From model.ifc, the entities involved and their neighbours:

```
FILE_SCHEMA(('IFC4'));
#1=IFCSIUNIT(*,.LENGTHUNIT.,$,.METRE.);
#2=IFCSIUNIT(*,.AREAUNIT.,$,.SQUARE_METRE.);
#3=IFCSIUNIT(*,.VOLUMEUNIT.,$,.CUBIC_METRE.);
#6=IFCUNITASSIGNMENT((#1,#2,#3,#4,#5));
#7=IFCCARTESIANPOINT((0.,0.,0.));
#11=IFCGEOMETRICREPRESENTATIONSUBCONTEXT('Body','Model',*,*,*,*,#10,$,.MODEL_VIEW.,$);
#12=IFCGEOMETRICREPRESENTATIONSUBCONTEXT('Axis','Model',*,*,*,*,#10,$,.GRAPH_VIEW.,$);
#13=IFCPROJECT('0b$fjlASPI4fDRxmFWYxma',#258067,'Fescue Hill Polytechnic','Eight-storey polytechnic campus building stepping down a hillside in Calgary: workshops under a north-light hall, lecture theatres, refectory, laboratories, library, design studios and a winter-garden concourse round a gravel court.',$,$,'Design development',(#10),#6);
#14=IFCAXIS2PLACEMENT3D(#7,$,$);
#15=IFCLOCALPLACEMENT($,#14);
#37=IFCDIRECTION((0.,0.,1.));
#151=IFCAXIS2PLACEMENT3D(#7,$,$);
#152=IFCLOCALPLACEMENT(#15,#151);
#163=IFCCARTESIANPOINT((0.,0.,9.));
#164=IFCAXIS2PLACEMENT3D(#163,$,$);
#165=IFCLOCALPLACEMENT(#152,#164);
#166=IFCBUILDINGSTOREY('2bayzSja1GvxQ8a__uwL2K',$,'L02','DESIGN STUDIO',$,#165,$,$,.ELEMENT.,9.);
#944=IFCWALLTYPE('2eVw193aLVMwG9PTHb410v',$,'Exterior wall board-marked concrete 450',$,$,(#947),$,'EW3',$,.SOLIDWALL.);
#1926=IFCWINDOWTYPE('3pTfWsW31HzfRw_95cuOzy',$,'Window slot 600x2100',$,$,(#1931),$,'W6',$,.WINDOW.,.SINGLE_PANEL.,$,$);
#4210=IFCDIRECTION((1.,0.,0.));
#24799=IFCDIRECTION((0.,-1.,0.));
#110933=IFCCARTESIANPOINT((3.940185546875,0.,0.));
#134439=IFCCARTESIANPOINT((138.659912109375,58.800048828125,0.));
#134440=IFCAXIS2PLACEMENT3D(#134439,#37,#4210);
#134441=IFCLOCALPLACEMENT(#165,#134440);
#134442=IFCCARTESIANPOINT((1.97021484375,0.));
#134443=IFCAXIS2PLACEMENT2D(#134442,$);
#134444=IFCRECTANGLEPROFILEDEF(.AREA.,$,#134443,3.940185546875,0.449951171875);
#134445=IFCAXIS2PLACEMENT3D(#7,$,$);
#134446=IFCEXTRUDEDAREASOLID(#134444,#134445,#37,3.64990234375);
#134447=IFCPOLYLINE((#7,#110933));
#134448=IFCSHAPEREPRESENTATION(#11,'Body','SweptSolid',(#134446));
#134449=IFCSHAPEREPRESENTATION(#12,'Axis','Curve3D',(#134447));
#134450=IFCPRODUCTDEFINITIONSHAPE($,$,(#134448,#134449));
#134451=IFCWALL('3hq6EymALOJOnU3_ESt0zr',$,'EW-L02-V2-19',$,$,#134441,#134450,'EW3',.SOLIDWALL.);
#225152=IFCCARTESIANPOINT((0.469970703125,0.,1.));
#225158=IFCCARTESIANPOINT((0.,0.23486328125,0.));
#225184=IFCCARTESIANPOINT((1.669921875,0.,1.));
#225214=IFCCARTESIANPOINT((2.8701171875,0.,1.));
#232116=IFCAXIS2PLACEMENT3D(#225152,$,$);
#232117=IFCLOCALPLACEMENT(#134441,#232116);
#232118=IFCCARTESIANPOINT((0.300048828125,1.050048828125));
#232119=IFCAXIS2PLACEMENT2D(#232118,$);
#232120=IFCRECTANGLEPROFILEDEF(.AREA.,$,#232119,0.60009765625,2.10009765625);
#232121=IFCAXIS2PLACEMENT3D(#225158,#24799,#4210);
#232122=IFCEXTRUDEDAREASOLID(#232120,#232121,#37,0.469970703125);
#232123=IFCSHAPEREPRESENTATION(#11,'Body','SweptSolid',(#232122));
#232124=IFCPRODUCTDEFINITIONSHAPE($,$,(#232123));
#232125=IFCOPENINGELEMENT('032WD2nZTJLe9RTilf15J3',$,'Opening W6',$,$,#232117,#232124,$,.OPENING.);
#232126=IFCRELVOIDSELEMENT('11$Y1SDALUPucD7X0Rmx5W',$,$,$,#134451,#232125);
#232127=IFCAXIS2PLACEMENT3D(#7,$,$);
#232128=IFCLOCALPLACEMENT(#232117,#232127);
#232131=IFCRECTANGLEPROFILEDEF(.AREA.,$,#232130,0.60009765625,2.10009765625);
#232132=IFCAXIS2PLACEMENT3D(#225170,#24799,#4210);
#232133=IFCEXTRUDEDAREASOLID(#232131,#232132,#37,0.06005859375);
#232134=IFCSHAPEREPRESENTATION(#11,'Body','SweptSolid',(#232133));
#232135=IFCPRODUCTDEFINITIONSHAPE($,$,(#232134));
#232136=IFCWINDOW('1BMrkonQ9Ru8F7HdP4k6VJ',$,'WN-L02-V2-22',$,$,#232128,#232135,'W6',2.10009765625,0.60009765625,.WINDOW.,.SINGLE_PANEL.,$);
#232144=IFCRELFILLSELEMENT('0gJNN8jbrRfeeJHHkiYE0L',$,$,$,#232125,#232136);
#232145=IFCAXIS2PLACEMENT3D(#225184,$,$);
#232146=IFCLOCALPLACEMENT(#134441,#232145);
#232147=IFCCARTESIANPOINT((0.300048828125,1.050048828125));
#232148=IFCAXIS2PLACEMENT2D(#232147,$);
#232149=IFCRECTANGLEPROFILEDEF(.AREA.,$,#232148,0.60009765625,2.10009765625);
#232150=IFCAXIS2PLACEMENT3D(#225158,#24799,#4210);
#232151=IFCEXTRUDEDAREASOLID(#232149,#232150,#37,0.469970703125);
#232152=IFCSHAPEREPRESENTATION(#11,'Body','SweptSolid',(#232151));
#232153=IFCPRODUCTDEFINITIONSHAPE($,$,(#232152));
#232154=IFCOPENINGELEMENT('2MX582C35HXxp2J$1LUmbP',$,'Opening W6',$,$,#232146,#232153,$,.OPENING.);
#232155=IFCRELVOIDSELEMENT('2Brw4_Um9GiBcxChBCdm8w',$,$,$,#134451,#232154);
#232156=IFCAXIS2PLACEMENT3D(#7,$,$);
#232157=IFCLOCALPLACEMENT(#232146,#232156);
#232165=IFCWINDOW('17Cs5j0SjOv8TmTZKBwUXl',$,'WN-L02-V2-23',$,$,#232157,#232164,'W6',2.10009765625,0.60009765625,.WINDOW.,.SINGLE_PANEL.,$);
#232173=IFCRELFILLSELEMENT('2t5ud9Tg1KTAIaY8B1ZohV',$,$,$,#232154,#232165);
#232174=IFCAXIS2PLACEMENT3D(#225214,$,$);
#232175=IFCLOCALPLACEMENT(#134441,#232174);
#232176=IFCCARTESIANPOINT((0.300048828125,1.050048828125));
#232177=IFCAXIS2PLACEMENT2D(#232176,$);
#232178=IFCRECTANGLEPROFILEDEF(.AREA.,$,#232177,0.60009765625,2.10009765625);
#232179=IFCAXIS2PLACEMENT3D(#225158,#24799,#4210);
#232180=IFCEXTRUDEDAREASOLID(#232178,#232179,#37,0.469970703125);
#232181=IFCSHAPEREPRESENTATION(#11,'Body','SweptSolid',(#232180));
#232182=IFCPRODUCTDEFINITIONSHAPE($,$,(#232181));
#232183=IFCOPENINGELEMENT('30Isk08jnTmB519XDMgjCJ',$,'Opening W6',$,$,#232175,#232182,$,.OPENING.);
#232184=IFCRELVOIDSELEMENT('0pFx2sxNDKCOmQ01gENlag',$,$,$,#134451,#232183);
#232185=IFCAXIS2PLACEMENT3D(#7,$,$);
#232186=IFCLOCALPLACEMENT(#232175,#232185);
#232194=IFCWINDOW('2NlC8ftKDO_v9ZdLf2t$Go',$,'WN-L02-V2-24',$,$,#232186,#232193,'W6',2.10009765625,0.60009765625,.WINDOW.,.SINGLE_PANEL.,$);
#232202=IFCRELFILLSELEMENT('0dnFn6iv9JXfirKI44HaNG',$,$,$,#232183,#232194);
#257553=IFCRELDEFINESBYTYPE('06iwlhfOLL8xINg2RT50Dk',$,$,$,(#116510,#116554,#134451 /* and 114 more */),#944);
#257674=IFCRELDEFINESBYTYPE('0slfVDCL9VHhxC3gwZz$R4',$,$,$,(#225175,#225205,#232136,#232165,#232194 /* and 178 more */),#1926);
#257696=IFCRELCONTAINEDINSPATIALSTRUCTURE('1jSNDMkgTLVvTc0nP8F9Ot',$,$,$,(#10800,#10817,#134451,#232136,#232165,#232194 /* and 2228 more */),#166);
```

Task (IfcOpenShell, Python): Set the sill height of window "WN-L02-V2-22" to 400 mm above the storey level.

```python
import numpy as np
import ifcopenshell
import ifcopenshell.api.geometry
import ifcopenshell.geom
import ifcopenshell.util.element
import ifcopenshell.util.placement
import ifcopenshell.util.shape
import ifcopenshell.util.unit

model = ifcopenshell.open("model.ifc")
unit_scale = ifcopenshell.util.unit.calculate_unit_scale(model)

window = model.by_id(232136)
opening = window.FillsVoids[0].RelatingOpeningElement
storey = ifcopenshell.util.element.get_container(window, ifc_class="IfcBuildingStorey")
level = ifcopenshell.util.placement.get_local_placement(storey.ObjectPlacement)[2, 3]

# The opening's origin need not be at the sill, so measure its lowest point.
shape = ifcopenshell.geom.create_shape(ifcopenshell.geom.settings(), opening)
bottom = ifcopenshell.util.shape.get_shape_bottom_elevation(shape, shape.geometry) / unit_scale
dz = level + 0.4 / unit_scale - bottom

shift = np.array([0.0, 0.0, dz])
# The window is placed relative to its opening, so it follows when the opening moves.
matrix = ifcopenshell.util.placement.get_local_placement(opening.ObjectPlacement)
matrix[:3, 3] += shift
ifcopenshell.api.geometry.edit_object_placement(
    model, product=opening, matrix=matrix, is_si=False, should_transform_children=True
)

print(f"moved by {dz * unit_scale:+.3f} m")

model.write("model_edited.ifc")
```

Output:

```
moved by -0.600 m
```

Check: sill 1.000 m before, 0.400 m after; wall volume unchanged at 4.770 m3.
